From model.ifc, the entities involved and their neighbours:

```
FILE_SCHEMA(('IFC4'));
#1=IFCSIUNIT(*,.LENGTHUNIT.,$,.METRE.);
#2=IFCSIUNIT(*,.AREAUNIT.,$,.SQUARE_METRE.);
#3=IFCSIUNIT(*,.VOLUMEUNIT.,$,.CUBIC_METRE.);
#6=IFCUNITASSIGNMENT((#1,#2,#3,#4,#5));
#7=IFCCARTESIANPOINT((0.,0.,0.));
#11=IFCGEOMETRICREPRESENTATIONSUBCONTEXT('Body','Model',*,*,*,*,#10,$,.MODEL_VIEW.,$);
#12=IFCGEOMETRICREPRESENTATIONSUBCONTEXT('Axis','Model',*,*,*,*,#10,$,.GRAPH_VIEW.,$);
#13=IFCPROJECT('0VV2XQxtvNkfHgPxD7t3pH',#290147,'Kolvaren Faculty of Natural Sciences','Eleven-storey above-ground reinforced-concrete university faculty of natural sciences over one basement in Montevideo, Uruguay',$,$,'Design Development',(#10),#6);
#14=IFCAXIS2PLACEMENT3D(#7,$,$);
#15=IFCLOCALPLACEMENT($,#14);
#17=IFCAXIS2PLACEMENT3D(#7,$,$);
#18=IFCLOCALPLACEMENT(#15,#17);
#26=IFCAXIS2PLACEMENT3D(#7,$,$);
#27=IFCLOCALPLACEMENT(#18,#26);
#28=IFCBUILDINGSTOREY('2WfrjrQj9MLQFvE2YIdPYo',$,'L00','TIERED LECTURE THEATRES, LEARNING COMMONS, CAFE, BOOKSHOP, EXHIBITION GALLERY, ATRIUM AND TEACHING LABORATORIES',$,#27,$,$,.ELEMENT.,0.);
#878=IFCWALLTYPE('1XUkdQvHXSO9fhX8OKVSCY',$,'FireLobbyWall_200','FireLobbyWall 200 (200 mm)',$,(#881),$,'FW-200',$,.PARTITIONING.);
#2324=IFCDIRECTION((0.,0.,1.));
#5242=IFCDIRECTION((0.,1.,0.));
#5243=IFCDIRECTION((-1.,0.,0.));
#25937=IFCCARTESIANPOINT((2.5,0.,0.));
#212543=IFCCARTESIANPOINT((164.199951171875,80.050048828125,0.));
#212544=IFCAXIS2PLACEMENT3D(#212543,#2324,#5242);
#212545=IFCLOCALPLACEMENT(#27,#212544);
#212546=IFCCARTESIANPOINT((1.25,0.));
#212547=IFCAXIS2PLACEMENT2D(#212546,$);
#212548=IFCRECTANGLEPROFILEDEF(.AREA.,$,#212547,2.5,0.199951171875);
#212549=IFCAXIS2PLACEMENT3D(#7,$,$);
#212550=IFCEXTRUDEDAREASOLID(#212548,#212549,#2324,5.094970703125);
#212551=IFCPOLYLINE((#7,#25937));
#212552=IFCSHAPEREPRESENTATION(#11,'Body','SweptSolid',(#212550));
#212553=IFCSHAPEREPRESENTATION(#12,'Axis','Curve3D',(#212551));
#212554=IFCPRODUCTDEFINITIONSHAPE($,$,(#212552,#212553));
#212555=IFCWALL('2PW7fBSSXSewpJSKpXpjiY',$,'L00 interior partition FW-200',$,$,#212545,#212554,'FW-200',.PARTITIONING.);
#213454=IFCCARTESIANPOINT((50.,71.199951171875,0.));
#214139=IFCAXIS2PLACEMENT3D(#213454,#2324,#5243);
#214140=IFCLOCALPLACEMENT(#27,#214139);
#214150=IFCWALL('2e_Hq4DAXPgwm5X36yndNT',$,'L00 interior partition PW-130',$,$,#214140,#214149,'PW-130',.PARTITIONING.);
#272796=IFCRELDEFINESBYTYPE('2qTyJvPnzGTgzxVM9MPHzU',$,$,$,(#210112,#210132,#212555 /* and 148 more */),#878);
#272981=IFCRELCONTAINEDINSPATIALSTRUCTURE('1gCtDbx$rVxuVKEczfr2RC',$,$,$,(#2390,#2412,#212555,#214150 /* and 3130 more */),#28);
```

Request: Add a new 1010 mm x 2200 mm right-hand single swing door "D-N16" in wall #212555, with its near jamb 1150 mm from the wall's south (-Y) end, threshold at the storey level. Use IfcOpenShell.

```python
import numpy as np
import ifcopenshell
import ifcopenshell.api.feature
import ifcopenshell.api.geometry
import ifcopenshell.api.root
import ifcopenshell.api.spatial
import ifcopenshell.geom
import ifcopenshell.util.element
import ifcopenshell.util.placement
import ifcopenshell.util.representation
import ifcopenshell.util.shape
import ifcopenshell.util.unit

model = ifcopenshell.open("model.ifc")
unit_scale = ifcopenshell.util.unit.calculate_unit_scale(model)
settings = ifcopenshell.geom.settings()


def volume(element):
    """Net volume in cubic metres, openings subtracted."""
    shape = ifcopenshell.geom.create_shape(settings, element)
    return ifcopenshell.util.shape.get_volume(shape.geometry)


wall = model.by_id(212555)
storey = ifcopenshell.util.element.get_container(wall, ifc_class="IfcBuildingStorey")
context = ifcopenshell.util.representation.get_context(model, "Model", "Body", "MODEL_VIEW")
before = volume(wall)

width, height, from_end, sill = 1.01, 2.2, 1.15, 0.0  # metres

# The wall runs along its own X axis, and the end named is its -X end.
wall_shape = ifcopenshell.geom.create_shape(settings, wall)
x, y, z = ifcopenshell.util.shape.get_vertices(wall_shape.geometry).T
start = x.min() + from_end
face, thickness = float(y.min()), float(y.max() - y.min())
wall_matrix = ifcopenshell.util.placement.get_local_placement(wall.ObjectPlacement)
level = ifcopenshell.util.placement.get_local_placement(storey.ObjectPlacement)[2, 3]


def in_wall(x, y):
    """Placement at x, y metres in the wall's axes, at sill height."""
    matrix = wall_matrix.copy()
    matrix[:, 3] = wall_matrix @ np.array([x / unit_scale, y / unit_scale, 0.0, 1.0])
    matrix[2, 3] = level + sill / unit_scale
    return matrix


# Opening: a box that overshoots both wall faces by 50 mm.
opening = ifcopenshell.api.root.create_entity(model, ifc_class="IfcOpeningElement", predefined_type="OPENING")
box = ifcopenshell.api.geometry.add_wall_representation(
    model, context=context, length=width, height=height, thickness=thickness + 0.1
)
ifcopenshell.api.geometry.assign_representation(model, product=opening, representation=box)
ifcopenshell.api.geometry.edit_object_placement(model, product=opening, matrix=in_wall(start, face - 0.05), is_si=False)
ifcopenshell.api.feature.add_feature(model, feature=opening, element=wall)

door = ifcopenshell.api.root.create_entity(model, ifc_class="IfcDoor", name="D-N16", predefined_type="DOOR")
door.OverallWidth, door.OverallHeight = width / unit_scale, height / unit_scale
door.OperationType = "SINGLE_SWING_RIGHT"
body = ifcopenshell.api.geometry.add_door_representation(
    model,
    context=context,
    overall_width=door.OverallWidth,
    overall_height=door.OverallHeight,
    operation_type="SINGLE_SWING_RIGHT",
    lining_properties={"LiningDepth": thickness / unit_scale, "ThresholdDepth": thickness / unit_scale},
)
ifcopenshell.api.geometry.assign_representation(model, product=door, representation=body)
ifcopenshell.api.spatial.assign_container(model, products=[door], relating_structure=storey)
ifcopenshell.api.feature.add_filling(model, opening=opening, element=door)

# The lining spans the wall, so the door starts at the wall face.
ifcopenshell.api.geometry.edit_object_placement(model, product=door, matrix=in_wall(start, face), is_si=False)

after = volume(wall)

print(f"wall volume {before:.3f} -> {after:.3f} m3")

model.write("model_rev.ifc")
```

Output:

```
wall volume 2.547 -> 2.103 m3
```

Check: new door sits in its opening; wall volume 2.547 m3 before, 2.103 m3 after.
